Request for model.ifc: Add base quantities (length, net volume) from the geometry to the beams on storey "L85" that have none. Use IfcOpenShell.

First a look at what the model holds.

```python
import ifcopenshell
import ifcopenshell.util.element
import ifcopenshell.util.unit

model = ifcopenshell.open("model.ifc")
print(model.schema)
for unit_type in ("LENGTHUNIT", "AREAUNIT", "VOLUMEUNIT"):
    print(unit_type, ifcopenshell.util.unit.calculate_unit_scale(model, unit_type))
storey = next(s for s in model.by_type("IfcBuildingStorey") if s.Name == "L85")
beams = [e for e in ifcopenshell.util.element.get_decomposition(storey) if e.is_a("IfcBeam")]
for e in sorted(beams, key=lambda e: e.id()):
    print(e.id(), e.is_a(), e.Name, list(ifcopenshell.util.element.get_psets(e, qtos_only=True)), sep=" | ")
```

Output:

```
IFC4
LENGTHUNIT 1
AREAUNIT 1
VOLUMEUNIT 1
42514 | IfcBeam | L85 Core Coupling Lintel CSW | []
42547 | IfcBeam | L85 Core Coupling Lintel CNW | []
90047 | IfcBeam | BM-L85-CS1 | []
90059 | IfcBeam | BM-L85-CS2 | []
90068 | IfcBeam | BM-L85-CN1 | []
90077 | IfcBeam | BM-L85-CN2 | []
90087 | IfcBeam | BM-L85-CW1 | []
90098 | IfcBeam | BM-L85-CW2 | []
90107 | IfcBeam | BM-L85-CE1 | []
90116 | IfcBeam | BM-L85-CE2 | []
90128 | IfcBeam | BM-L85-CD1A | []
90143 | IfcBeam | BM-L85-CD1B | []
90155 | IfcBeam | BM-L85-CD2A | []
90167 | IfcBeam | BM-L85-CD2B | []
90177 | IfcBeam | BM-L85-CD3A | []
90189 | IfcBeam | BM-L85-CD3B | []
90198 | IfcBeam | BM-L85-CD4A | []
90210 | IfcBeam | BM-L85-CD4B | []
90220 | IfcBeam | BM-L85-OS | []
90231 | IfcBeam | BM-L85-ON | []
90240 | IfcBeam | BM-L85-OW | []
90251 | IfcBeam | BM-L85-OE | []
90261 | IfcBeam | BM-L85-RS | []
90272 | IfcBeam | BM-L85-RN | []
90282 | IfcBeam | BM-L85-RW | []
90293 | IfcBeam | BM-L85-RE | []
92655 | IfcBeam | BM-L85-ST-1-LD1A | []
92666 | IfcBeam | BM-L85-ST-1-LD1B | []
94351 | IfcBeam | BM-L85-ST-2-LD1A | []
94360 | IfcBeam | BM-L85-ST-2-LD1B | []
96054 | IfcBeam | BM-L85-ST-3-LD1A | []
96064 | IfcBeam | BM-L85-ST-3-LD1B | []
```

```python
import ifcopenshell
import ifcopenshell.api.pset
import ifcopenshell.geom
import ifcopenshell.util.element
import ifcopenshell.util.shape
import ifcopenshell.util.unit

model = ifcopenshell.open("model.ifc")
unit_scale = ifcopenshell.util.unit.calculate_unit_scale(model)
volume_scale = ifcopenshell.util.unit.calculate_unit_scale(model, "VOLUMEUNIT")
settings = ifcopenshell.geom.settings()

storey = next(s for s in model.by_type("IfcBuildingStorey") if s.Name == "L85")
beams = [e for e in ifcopenshell.util.element.get_decomposition(storey) if e.is_a("IfcBeam")]

for e in sorted(beams, key=lambda e: e.id()):
    if ifcopenshell.util.element.get_psets(e, qtos_only=True, should_inherit=False):
        continue
    # Geometry comes back in metres, in the element's own axes.
    shape = ifcopenshell.geom.create_shape(settings, e)
    values = {
        "Length": ifcopenshell.util.shape.get_max_xyz(shape.geometry) / unit_scale,
        "NetVolume": ifcopenshell.util.shape.get_volume(shape.geometry) / volume_scale,
    }
    qto = ifcopenshell.api.pset.add_qto(model, product=e, name="Qto_BeamBaseQuantities")
    ifcopenshell.api.pset.edit_qto(model, qto=qto, properties=values)
    print(e.id(), {k: round(v, 3) for k, v in values.items()})

model.write("model_updated.ifc")
```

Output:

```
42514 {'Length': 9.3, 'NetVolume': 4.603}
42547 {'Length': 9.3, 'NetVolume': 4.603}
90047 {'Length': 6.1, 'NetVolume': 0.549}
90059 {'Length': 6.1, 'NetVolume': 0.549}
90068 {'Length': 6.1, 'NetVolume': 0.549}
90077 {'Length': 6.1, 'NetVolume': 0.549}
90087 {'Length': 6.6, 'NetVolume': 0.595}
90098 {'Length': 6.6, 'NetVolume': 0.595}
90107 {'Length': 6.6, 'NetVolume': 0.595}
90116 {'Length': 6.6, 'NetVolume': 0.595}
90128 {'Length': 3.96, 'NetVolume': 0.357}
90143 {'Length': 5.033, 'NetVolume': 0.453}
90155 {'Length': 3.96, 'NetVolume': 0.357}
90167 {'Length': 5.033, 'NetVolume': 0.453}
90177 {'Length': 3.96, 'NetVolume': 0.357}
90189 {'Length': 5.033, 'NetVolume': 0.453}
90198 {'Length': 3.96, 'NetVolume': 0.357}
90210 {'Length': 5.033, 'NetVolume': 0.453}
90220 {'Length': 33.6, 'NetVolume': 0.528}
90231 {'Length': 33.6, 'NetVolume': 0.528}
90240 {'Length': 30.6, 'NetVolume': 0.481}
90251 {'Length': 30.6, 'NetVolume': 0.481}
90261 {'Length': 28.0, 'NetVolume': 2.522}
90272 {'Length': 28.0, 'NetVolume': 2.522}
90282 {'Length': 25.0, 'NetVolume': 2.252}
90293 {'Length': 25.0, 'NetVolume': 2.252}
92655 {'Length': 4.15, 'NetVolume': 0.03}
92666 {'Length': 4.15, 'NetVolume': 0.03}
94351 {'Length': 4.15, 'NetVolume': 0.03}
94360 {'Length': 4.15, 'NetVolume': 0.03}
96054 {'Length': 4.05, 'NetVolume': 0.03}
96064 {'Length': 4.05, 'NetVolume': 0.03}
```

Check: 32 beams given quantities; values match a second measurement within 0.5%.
